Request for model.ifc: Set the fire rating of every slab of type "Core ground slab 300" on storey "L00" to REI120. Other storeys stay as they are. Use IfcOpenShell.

First a look at what the model holds.

```python
import ifcopenshell
import ifcopenshell.util.element

model = ifcopenshell.open("model.ifc")
print(model.schema)
storey = next(s for s in model.by_type("IfcBuildingStorey") if s.Name == "L00")
slabs = [e for e in ifcopenshell.util.element.get_decomposition(storey) if e.is_a("IfcSlab")]
seen = {}
for e in slabs:
    element_type = ifcopenshell.util.element.get_type(e)
    key = (element_type.Name if element_type != e and element_type else None, ifcopenshell.util.element.get_pset(e, "Pset_SlabCommon", "FireRating"))
    seen[key] = seen.get(key, 0) + 1
for (name, value), count in sorted(seen.items(), key=str):
    print(count, "x", name, "|", value)
```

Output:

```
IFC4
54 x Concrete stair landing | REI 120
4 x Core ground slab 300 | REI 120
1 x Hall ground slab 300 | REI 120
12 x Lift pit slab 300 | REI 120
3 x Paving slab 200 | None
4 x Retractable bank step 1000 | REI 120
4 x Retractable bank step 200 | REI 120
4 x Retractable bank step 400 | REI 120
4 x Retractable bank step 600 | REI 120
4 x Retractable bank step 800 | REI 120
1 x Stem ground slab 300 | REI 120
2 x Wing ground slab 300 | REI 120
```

```python
import ifcopenshell
import ifcopenshell.api.pset
import ifcopenshell.util.element

model = ifcopenshell.open("model.ifc")

storey = next(s for s in model.by_type("IfcBuildingStorey") if s.Name == "L00")
slabs = [e for e in ifcopenshell.util.element.get_decomposition(storey) if e.is_a("IfcSlab")]

count = 0
for e in slabs:
    element_type = ifcopenshell.util.element.get_type(e)
    if element_type in (None, e) or element_type.Name != "Core ground slab 300":
        continue
    # add_pset returns the element's existing set when there is one.
    pset = ifcopenshell.api.pset.add_pset(model, product=e, name="Pset_SlabCommon")
    ifcopenshell.api.pset.edit_pset(model, pset=pset, properties={"FireRating": "REI120"})
    count += 1

print(count, "slabs updated")

model.write("model-out.ifc")
```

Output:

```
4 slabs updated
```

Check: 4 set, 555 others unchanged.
